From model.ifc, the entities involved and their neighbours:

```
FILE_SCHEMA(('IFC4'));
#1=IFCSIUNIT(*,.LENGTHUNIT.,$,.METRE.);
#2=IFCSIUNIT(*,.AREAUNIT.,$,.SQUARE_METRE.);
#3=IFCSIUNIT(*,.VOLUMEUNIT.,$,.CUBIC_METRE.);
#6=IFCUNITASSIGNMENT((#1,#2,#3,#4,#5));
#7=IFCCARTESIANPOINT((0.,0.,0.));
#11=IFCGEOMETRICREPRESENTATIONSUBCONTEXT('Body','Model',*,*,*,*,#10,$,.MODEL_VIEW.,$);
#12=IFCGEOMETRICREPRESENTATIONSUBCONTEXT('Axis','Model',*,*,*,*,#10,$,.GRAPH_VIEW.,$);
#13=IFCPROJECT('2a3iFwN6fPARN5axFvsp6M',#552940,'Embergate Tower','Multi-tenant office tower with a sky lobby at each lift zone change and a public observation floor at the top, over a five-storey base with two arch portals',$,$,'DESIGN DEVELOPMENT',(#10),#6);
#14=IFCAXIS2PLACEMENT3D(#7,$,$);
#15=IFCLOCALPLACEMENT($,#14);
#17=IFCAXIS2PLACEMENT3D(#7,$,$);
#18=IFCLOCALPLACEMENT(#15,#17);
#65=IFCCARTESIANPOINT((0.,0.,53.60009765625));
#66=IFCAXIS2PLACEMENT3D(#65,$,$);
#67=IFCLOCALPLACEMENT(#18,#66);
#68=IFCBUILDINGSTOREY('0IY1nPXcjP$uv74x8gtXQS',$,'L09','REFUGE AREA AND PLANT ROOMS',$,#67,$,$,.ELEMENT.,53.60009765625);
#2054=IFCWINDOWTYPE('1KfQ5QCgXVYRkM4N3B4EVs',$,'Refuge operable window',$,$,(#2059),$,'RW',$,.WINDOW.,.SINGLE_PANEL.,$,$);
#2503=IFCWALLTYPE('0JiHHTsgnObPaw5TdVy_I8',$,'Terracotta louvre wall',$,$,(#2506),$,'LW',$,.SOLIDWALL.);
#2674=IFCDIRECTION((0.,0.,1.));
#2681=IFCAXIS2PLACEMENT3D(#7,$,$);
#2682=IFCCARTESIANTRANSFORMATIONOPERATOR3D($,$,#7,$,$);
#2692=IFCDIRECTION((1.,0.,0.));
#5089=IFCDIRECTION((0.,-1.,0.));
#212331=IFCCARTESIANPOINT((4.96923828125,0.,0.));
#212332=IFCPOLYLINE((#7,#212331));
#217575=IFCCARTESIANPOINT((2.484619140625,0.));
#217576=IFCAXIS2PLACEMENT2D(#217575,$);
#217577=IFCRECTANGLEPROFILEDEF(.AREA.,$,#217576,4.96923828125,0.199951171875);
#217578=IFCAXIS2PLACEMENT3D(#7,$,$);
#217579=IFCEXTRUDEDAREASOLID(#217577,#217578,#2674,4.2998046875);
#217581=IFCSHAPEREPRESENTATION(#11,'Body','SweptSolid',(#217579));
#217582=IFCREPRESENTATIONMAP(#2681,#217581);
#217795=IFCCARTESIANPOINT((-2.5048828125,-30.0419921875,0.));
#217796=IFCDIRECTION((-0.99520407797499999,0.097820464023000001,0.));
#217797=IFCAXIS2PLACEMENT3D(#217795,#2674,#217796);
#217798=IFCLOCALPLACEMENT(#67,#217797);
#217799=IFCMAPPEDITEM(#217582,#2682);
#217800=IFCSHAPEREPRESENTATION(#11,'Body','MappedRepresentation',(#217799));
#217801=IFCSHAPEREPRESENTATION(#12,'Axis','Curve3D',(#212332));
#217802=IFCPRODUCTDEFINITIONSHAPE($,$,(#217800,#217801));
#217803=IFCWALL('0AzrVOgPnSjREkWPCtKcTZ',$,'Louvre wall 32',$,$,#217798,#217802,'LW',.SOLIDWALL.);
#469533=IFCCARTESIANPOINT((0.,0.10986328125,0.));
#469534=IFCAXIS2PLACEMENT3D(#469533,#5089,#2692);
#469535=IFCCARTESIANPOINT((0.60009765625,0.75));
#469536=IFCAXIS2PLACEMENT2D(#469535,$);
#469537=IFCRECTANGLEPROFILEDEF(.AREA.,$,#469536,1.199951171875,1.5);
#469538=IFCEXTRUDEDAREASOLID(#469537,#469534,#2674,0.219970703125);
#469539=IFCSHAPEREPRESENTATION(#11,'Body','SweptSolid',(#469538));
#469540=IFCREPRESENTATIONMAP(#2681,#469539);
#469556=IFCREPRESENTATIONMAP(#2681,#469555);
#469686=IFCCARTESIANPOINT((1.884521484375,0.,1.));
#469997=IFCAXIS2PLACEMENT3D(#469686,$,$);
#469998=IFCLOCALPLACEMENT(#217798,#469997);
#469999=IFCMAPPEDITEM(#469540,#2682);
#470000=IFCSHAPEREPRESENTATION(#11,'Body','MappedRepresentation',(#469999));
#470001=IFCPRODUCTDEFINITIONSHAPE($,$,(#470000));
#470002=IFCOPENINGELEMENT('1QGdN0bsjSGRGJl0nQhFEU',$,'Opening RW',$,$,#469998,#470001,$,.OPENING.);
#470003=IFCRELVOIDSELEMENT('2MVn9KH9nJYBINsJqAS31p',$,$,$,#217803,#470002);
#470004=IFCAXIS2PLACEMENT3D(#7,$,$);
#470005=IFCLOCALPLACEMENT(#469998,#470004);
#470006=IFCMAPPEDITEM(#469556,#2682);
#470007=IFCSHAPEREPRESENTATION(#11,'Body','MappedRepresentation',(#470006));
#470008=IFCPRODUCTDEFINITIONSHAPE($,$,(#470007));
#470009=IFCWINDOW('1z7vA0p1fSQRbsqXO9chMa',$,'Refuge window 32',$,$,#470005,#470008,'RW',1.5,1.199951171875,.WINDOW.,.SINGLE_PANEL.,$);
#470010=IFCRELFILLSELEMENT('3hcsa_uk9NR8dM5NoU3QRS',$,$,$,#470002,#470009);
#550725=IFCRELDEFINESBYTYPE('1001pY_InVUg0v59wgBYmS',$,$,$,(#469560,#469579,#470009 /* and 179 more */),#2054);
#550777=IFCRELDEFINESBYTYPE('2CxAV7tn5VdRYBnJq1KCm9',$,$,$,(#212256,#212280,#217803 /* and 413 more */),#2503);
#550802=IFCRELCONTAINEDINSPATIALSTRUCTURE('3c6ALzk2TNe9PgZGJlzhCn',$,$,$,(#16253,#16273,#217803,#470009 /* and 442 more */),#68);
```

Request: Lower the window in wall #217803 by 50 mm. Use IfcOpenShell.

```python
import numpy as np
import ifcopenshell
import ifcopenshell.api.geometry
import ifcopenshell.util.placement
import ifcopenshell.util.unit

model = ifcopenshell.open("model.ifc")
unit_scale = ifcopenshell.util.unit.calculate_unit_scale(model)

window = model.by_guid("1z7vA0p1fSQRbsqXO9chMa")
opening = window.FillsVoids[0].RelatingOpeningElement
dz = -0.05 / unit_scale

shift = np.array([0.0, 0.0, dz])
# The window is placed relative to its opening, so it follows when the opening moves.
matrix = ifcopenshell.util.placement.get_local_placement(opening.ObjectPlacement)
matrix[:3, 3] += shift
ifcopenshell.api.geometry.edit_object_placement(
    model, product=opening, matrix=matrix, is_si=False, should_transform_children=True
)

print(f"moved by {dz * unit_scale:+.3f} m")

model.write("model_updated.ifc")
```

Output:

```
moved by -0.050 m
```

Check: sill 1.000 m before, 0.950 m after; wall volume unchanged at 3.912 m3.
